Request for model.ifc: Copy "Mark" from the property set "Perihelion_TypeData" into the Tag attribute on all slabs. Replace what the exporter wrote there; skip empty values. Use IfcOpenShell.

First a look at what the model holds.

```python
import ifcopenshell
import ifcopenshell.util.element

model = ifcopenshell.open("model.ifc")
print(model.schema)
slabs = model.by_type("IfcSlab")
print(len(slabs), "slabs")
for e in slabs[:8]:
    source = ifcopenshell.util.element.get_pset(e, "Perihelion_TypeData", "Mark")
    target = e.Tag
    print(e.id(), repr(source), repr(target), sep=" | ")
```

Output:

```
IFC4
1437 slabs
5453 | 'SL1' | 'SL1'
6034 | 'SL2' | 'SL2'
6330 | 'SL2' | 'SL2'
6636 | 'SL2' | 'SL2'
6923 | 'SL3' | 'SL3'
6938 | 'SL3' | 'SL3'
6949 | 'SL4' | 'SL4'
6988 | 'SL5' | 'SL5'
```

```python
import ifcopenshell
import ifcopenshell.util.element

model = ifcopenshell.open("model.ifc")

count = 0
for e in model.by_type("IfcSlab"):
    value = ifcopenshell.util.element.get_pset(e, "Perihelion_TypeData", "Mark")
    current = e.Tag
    if not value or not value.strip() or current == value:
        continue
    e.Tag = value
    count += 1

print(count, "slabs updated")

model.write("model_rev.ifc")
```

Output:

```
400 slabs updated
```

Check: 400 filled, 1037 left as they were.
